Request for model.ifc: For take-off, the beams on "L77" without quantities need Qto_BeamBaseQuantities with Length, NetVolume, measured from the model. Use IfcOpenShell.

First a look at what the model holds.

```python
import ifcopenshell
import ifcopenshell.util.element
import ifcopenshell.util.unit

model = ifcopenshell.open("model.ifc")
print(model.schema)
for unit_type in ("LENGTHUNIT", "AREAUNIT", "VOLUMEUNIT"):
    print(unit_type, ifcopenshell.util.unit.calculate_unit_scale(model, unit_type))
storey = next(s for s in model.by_type("IfcBuildingStorey") if s.Name == "L77")
beams = [e for e in ifcopenshell.util.element.get_decomposition(storey) if e.is_a("IfcBeam")]
for e in sorted(beams, key=lambda e: e.id()):
    print(e.id(), e.is_a(), e.Name, list(ifcopenshell.util.element.get_psets(e, qtos_only=True)), sep=" | ")
```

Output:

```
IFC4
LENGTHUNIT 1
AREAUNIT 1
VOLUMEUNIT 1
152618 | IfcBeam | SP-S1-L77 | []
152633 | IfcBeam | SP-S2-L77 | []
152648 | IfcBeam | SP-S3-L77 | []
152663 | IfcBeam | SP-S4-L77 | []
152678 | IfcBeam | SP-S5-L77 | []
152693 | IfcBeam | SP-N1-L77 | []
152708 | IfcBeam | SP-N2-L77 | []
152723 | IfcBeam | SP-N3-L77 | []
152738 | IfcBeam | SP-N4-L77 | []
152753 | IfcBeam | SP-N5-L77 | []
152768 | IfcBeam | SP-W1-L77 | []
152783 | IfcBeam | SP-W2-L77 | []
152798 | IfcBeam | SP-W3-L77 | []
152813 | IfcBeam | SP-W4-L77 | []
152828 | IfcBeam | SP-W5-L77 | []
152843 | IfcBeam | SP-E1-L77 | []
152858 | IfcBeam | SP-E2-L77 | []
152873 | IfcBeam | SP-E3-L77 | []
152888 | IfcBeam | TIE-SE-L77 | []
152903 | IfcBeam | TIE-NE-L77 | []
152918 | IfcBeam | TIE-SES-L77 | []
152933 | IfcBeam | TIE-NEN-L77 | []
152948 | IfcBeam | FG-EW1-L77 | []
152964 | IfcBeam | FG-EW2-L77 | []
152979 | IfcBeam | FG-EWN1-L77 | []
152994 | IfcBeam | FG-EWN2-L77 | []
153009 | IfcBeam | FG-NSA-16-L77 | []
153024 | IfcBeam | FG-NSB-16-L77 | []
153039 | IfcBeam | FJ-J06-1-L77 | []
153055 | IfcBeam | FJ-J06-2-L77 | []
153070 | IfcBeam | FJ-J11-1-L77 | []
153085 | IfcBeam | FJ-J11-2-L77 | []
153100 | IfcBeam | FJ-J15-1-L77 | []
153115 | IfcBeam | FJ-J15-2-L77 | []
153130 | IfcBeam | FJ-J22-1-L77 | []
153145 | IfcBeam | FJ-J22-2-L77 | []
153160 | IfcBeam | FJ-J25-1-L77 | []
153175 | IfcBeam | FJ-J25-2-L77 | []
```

```python
import ifcopenshell
import ifcopenshell.api.pset
import ifcopenshell.geom
import ifcopenshell.util.element
import ifcopenshell.util.shape
import ifcopenshell.util.unit

model = ifcopenshell.open("model.ifc")
unit_scale = ifcopenshell.util.unit.calculate_unit_scale(model)
volume_scale = ifcopenshell.util.unit.calculate_unit_scale(model, "VOLUMEUNIT")
settings = ifcopenshell.geom.settings()

storey = next(s for s in model.by_type("IfcBuildingStorey") if s.Name == "L77")
beams = [e for e in ifcopenshell.util.element.get_decomposition(storey) if e.is_a("IfcBeam")]

for e in sorted(beams, key=lambda e: e.id()):
    if ifcopenshell.util.element.get_psets(e, qtos_only=True, should_inherit=False):
        continue
    # Geometry comes back in metres, in the element's own axes.
    shape = ifcopenshell.geom.create_shape(settings, e)
    values = {
        "Length": ifcopenshell.util.shape.get_max_xyz(shape.geometry) / unit_scale,
        "NetVolume": ifcopenshell.util.shape.get_volume(shape.geometry) / volume_scale,
    }
    qto = ifcopenshell.api.pset.add_qto(model, product=e, name="Qto_BeamBaseQuantities")
    ifcopenshell.api.pset.edit_qto(model, qto=qto, properties=values)
    print(e.id(), {k: round(v, 3) for k, v in values.items()})

model.write("model-out.ifc")
```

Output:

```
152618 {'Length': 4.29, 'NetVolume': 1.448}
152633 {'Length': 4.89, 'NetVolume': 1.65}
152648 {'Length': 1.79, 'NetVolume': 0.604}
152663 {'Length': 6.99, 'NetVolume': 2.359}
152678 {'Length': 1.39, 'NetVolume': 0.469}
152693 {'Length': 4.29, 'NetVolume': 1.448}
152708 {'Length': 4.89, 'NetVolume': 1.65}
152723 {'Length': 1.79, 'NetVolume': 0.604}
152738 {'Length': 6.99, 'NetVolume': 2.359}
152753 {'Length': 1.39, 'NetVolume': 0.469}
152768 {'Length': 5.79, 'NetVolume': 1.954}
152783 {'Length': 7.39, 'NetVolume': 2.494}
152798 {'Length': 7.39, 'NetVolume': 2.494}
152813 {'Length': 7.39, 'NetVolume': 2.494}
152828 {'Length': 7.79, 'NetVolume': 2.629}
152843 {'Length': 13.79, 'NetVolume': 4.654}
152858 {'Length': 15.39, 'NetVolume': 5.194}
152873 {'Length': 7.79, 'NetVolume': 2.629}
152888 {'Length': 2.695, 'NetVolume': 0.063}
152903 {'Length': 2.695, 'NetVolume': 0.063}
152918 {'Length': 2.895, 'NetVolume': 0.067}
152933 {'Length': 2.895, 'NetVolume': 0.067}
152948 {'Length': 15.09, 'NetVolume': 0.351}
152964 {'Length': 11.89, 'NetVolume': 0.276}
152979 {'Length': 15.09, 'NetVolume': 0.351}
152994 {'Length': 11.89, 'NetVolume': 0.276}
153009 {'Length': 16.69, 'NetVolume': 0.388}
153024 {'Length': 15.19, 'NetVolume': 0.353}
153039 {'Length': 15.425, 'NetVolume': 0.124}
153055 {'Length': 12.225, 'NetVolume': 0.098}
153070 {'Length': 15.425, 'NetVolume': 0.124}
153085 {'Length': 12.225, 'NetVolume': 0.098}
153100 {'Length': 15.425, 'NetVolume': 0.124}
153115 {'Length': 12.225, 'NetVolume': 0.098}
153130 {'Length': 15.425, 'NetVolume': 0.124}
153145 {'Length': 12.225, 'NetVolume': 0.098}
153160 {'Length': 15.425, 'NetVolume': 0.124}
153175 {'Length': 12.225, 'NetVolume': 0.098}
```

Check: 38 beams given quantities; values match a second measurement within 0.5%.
